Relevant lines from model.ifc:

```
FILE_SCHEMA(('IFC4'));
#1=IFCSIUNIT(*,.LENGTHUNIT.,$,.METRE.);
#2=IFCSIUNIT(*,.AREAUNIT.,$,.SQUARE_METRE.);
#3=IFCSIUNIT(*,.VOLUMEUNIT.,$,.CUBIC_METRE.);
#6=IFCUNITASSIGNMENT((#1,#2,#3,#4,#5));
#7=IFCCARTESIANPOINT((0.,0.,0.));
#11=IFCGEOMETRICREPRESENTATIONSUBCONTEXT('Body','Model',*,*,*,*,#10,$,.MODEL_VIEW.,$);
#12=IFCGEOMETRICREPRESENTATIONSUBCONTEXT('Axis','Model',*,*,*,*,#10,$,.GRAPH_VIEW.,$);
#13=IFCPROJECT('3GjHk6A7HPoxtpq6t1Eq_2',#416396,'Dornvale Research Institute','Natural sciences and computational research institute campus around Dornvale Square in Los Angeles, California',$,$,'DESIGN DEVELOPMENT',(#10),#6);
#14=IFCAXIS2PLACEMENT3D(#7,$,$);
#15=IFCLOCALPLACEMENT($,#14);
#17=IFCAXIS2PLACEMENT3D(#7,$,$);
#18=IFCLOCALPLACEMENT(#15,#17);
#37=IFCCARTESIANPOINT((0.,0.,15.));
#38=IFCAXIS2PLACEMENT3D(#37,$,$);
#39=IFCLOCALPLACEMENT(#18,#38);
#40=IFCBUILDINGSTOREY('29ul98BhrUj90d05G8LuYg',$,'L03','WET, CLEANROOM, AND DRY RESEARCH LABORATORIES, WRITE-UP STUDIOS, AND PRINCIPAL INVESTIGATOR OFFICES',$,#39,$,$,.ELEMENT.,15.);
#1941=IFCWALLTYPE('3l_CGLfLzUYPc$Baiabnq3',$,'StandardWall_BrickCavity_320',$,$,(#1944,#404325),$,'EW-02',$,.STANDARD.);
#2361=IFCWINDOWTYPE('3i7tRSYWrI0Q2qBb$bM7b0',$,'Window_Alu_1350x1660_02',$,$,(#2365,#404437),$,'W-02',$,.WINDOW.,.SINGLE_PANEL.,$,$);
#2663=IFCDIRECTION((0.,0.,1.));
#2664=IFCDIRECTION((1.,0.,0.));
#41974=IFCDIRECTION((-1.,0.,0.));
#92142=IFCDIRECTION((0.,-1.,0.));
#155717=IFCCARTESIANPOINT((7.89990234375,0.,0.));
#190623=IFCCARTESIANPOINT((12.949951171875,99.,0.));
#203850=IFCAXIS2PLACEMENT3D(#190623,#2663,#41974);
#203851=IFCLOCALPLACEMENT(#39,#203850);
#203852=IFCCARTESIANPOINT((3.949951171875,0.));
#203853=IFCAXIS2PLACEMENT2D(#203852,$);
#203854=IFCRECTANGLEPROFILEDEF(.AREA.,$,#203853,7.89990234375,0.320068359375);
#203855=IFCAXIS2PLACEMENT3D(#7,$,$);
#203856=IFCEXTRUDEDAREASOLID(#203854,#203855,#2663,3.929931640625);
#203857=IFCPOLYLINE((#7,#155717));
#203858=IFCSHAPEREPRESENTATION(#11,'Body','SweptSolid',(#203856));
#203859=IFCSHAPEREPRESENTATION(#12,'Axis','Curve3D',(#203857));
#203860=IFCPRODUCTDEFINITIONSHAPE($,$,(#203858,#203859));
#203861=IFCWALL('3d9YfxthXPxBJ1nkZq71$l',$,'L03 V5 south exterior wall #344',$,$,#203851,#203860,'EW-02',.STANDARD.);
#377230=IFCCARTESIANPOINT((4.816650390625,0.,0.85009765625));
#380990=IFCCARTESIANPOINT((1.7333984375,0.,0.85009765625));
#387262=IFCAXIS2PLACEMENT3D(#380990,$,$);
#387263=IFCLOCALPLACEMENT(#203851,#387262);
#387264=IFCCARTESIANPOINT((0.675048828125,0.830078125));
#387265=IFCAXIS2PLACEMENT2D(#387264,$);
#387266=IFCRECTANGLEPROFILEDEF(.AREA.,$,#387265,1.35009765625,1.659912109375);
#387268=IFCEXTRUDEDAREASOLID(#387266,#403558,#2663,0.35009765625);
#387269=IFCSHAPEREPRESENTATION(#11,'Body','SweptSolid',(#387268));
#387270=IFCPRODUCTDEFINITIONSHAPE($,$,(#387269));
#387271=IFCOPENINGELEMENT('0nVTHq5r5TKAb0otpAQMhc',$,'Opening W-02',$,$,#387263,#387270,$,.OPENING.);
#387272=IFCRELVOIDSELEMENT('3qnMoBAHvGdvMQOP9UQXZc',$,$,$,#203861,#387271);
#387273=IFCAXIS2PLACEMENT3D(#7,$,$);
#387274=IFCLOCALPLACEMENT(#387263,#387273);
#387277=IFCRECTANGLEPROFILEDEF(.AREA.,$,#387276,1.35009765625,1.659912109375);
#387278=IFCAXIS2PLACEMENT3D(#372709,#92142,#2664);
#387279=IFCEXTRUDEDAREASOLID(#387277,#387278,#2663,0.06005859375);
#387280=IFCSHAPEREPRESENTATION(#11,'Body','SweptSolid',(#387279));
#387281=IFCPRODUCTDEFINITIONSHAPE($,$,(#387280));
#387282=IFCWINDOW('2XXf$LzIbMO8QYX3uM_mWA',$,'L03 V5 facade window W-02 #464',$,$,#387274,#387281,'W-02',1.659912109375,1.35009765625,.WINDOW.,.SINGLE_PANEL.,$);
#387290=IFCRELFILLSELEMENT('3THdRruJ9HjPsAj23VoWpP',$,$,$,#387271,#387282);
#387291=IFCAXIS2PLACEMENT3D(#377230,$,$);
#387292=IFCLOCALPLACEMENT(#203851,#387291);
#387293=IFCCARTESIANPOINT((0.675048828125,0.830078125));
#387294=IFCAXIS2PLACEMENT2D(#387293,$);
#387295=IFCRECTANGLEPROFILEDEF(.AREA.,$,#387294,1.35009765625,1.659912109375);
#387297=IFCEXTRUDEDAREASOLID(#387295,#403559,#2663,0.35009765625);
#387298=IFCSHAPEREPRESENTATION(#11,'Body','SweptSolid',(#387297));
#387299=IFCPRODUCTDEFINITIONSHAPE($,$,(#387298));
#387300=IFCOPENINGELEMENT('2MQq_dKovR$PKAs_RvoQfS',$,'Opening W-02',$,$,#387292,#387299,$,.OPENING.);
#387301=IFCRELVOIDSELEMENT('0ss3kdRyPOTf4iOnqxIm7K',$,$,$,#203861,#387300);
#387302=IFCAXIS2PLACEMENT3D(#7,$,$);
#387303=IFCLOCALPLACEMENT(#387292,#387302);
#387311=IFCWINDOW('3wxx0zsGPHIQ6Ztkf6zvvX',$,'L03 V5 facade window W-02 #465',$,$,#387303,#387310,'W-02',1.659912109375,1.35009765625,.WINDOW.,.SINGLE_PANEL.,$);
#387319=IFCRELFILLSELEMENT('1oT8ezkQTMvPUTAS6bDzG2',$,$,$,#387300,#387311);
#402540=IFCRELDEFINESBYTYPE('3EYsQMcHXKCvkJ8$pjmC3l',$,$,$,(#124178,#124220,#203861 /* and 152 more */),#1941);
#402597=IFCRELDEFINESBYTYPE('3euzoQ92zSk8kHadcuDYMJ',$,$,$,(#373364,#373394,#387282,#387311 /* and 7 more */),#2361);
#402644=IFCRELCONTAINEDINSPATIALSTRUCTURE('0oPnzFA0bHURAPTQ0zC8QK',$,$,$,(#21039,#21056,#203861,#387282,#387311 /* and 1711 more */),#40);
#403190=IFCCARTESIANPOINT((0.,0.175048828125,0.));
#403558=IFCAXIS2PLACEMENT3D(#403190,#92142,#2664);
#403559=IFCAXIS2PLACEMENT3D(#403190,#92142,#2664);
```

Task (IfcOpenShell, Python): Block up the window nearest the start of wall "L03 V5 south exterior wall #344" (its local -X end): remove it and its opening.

```python
import ifcopenshell
import ifcopenshell.api.feature
import ifcopenshell.api.root
import ifcopenshell.geom
import ifcopenshell.util.shape

model = ifcopenshell.open("model.ifc")
settings = ifcopenshell.geom.settings()


def volume(element):
    """Net volume in cubic metres, openings subtracted."""
    shape = ifcopenshell.geom.create_shape(settings, element)
    return ifcopenshell.util.shape.get_volume(shape.geometry)


window = model.by_guid("2XXf$LzIbMO8QYX3uM_mWA")
opening = window.FillsVoids[0].RelatingOpeningElement
wall = opening.VoidsElements[0].RelatingBuildingElement
before = volume(wall)

ifcopenshell.api.root.remove_product(model, product=window)
ifcopenshell.api.feature.remove_feature(model, feature=opening)

after = volume(wall)

print(f"wall volume {before:.3f} -> {after:.3f} m3")

model.write("model-out.ifc")
```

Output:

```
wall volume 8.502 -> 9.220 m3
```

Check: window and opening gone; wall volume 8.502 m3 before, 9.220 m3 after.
